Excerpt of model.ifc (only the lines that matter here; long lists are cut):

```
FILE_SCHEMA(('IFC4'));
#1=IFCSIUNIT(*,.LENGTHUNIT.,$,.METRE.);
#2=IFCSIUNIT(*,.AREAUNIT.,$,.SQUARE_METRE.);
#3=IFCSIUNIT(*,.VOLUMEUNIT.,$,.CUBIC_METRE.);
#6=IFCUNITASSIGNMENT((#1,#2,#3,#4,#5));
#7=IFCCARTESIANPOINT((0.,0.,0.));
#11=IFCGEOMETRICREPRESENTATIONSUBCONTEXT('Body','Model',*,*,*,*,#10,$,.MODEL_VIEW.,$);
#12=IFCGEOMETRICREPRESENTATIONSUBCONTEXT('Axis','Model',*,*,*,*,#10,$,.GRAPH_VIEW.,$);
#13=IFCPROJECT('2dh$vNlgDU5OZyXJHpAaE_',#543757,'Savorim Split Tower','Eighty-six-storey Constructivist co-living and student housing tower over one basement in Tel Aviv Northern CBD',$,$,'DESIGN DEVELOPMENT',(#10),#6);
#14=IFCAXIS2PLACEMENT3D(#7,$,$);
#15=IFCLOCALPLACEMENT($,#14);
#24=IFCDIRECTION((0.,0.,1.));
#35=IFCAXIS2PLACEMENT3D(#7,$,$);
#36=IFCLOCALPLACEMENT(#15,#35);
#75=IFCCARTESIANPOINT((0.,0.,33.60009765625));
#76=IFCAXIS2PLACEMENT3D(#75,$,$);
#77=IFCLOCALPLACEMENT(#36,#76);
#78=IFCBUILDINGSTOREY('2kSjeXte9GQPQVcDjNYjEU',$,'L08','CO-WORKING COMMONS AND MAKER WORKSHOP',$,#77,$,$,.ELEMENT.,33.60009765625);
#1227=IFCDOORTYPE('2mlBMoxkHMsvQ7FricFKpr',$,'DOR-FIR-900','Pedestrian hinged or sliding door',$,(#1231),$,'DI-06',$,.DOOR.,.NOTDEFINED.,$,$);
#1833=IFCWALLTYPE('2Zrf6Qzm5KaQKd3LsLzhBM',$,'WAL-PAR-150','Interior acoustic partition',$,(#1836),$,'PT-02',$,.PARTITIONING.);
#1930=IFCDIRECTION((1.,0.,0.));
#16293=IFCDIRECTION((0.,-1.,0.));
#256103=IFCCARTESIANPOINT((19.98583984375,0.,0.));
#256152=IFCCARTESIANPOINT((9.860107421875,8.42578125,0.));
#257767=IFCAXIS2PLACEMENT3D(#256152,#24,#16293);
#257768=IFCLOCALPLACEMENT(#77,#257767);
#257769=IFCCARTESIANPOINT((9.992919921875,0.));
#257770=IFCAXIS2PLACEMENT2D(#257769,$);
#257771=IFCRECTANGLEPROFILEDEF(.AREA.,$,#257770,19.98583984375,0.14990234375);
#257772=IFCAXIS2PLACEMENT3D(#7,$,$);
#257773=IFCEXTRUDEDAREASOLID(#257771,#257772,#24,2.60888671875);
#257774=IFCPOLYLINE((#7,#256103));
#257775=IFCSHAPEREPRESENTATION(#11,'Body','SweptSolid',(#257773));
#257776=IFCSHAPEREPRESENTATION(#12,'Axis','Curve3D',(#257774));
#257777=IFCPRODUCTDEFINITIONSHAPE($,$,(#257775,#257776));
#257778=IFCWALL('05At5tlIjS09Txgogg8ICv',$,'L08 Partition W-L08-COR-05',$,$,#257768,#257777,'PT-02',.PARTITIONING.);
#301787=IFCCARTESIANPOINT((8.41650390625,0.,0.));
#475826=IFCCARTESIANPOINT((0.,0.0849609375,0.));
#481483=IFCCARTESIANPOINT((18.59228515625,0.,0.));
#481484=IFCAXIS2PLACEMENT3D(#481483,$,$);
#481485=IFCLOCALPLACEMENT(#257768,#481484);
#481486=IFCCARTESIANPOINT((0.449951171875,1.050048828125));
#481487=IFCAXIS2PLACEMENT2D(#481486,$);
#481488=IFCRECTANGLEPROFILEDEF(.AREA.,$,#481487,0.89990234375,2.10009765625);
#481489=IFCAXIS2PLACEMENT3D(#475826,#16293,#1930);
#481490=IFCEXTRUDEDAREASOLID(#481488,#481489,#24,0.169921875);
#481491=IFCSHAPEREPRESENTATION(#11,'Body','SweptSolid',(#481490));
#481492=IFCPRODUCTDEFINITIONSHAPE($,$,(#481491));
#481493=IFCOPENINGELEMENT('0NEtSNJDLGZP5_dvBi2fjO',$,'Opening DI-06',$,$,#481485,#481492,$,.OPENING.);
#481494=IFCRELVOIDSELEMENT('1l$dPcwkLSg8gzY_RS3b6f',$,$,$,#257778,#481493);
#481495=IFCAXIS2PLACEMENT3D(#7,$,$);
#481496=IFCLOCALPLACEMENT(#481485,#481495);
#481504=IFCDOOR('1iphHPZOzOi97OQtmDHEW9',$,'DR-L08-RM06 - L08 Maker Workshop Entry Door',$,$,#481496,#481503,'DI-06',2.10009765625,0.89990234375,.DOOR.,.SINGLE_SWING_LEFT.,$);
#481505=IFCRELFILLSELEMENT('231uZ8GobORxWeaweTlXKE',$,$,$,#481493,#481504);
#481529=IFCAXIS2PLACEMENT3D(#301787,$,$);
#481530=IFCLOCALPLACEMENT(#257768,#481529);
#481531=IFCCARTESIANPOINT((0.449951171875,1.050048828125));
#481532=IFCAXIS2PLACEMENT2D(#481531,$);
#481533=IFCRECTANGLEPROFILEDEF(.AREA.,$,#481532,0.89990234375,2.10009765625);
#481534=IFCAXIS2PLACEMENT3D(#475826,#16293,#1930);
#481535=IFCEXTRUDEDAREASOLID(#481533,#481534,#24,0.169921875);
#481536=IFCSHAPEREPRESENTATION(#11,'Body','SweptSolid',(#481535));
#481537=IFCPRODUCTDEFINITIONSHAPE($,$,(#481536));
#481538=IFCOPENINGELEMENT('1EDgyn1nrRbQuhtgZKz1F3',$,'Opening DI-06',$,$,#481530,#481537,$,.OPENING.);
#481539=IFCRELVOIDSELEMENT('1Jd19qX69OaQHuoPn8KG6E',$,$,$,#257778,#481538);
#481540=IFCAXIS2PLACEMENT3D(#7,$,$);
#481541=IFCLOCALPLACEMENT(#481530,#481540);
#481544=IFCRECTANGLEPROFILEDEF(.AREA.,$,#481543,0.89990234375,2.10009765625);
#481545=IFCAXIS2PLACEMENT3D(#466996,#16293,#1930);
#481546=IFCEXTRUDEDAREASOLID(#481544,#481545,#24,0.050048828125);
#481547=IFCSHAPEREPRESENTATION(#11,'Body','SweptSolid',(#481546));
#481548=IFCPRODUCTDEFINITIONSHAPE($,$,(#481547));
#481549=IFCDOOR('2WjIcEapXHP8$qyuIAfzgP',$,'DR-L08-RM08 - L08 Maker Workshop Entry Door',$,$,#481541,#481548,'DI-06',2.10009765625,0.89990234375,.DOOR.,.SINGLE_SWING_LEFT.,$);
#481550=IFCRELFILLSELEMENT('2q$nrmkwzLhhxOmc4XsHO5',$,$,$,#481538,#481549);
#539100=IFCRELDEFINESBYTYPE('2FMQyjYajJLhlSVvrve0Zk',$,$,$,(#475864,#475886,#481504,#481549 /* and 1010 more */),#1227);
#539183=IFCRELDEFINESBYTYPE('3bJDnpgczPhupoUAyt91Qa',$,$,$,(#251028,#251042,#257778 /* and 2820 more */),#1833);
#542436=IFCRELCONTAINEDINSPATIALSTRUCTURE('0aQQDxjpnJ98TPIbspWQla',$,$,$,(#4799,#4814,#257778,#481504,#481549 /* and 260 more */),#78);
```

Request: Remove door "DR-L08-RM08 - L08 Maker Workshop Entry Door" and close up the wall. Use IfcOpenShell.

```python
import ifcopenshell
import ifcopenshell.api.feature
import ifcopenshell.api.root
import ifcopenshell.geom
import ifcopenshell.util.shape

model = ifcopenshell.open("model.ifc")
settings = ifcopenshell.geom.settings()


def volume(element):
    """Net volume in cubic metres, openings subtracted."""
    shape = ifcopenshell.geom.create_shape(settings, element)
    return ifcopenshell.util.shape.get_volume(shape.geometry)


door = model.by_id(481549)
opening = door.FillsVoids[0].RelatingOpeningElement
wall = opening.VoidsElements[0].RelatingBuildingElement
before = volume(wall)

ifcopenshell.api.root.remove_product(model, product=door)
ifcopenshell.api.feature.remove_feature(model, feature=opening)

after = volume(wall)

print(f"wall volume {before:.3f} -> {after:.3f} m3")

model.write("model_v2.ifc")
```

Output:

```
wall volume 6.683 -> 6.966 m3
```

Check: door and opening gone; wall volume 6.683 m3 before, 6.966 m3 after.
